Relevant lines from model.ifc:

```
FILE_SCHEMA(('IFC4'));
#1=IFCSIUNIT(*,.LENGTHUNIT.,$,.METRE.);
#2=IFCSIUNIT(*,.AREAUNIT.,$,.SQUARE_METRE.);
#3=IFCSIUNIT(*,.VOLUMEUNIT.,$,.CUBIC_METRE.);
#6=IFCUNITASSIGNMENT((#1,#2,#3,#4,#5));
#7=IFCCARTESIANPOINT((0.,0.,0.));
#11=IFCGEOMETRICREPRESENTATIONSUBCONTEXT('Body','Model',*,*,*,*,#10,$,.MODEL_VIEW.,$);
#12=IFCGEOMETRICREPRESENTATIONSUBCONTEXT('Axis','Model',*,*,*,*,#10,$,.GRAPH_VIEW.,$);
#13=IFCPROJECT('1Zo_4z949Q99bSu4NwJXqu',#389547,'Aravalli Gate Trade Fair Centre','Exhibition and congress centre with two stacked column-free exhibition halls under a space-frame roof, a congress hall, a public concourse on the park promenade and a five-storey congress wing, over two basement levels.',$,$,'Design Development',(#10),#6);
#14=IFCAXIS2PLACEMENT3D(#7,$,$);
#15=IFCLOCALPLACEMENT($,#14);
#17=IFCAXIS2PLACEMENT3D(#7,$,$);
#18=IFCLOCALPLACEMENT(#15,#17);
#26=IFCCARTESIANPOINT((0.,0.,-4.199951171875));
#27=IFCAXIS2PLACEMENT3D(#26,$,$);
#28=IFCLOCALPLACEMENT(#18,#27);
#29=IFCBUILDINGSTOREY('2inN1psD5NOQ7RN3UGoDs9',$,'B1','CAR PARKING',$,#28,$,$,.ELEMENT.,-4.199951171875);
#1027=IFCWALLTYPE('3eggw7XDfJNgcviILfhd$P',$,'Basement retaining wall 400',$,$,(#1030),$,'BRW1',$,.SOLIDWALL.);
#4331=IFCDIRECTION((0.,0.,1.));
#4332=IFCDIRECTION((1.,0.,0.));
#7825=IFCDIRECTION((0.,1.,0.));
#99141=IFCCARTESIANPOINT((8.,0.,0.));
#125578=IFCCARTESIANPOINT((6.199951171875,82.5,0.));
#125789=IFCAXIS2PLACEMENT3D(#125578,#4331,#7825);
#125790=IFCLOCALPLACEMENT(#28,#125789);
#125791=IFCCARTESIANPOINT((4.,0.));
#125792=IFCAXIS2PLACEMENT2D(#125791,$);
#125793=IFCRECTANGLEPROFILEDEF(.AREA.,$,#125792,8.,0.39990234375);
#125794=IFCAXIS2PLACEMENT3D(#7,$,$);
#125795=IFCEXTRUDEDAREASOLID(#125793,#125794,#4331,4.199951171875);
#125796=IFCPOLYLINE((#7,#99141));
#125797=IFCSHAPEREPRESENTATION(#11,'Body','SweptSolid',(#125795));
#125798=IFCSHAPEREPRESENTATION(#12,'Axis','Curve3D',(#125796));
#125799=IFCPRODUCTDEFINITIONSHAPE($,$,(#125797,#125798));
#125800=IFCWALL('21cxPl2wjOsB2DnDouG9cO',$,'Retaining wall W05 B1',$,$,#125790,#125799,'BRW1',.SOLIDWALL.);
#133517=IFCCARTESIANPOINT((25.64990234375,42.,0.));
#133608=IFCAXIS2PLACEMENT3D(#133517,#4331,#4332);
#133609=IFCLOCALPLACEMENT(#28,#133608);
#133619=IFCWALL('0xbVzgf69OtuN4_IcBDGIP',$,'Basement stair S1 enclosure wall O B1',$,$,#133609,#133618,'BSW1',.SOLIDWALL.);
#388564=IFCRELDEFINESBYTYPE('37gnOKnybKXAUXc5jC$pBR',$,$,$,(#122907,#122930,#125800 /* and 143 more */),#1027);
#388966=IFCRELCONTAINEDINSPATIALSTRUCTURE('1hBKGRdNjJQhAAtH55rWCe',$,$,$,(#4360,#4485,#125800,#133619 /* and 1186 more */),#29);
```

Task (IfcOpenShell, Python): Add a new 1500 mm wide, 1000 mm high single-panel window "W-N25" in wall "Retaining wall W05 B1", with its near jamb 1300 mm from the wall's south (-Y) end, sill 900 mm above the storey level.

```python
import numpy as np
import ifcopenshell
import ifcopenshell.api.feature
import ifcopenshell.api.geometry
import ifcopenshell.api.root
import ifcopenshell.api.spatial
import ifcopenshell.geom
import ifcopenshell.util.element
import ifcopenshell.util.placement
import ifcopenshell.util.representation
import ifcopenshell.util.shape
import ifcopenshell.util.unit

model = ifcopenshell.open("model.ifc")
unit_scale = ifcopenshell.util.unit.calculate_unit_scale(model)
settings = ifcopenshell.geom.settings()


def volume(element):
    """Net volume in cubic metres, openings subtracted."""
    shape = ifcopenshell.geom.create_shape(settings, element)
    return ifcopenshell.util.shape.get_volume(shape.geometry)


wall = model.by_guid("21cxPl2wjOsB2DnDouG9cO")
storey = ifcopenshell.util.element.get_container(wall, ifc_class="IfcBuildingStorey")
context = ifcopenshell.util.representation.get_context(model, "Model", "Body", "MODEL_VIEW")
before = volume(wall)

width, height, from_end, sill = 1.5, 1, 1.3, 0.9  # metres

# The wall runs along its own X axis, and the end named is its -X end.
wall_shape = ifcopenshell.geom.create_shape(settings, wall)
x, y, z = ifcopenshell.util.shape.get_vertices(wall_shape.geometry).T
start = x.min() + from_end
face, thickness = float(y.min()), float(y.max() - y.min())
wall_matrix = ifcopenshell.util.placement.get_local_placement(wall.ObjectPlacement)
level = ifcopenshell.util.placement.get_local_placement(storey.ObjectPlacement)[2, 3]


def in_wall(x, y):
    """Placement at x, y metres in the wall's axes, at sill height."""
    matrix = wall_matrix.copy()
    matrix[:, 3] = wall_matrix @ np.array([x / unit_scale, y / unit_scale, 0.0, 1.0])
    matrix[2, 3] = level + sill / unit_scale
    return matrix


# Opening: a box that overshoots both wall faces by 50 mm.
opening = ifcopenshell.api.root.create_entity(model, ifc_class="IfcOpeningElement", predefined_type="OPENING")
box = ifcopenshell.api.geometry.add_wall_representation(
    model, context=context, length=width, height=height, thickness=thickness + 0.1
)
ifcopenshell.api.geometry.assign_representation(model, product=opening, representation=box)
ifcopenshell.api.geometry.edit_object_placement(model, product=opening, matrix=in_wall(start, face - 0.05), is_si=False)
ifcopenshell.api.feature.add_feature(model, feature=opening, element=wall)

window = ifcopenshell.api.root.create_entity(model, ifc_class="IfcWindow", name="W-N25", predefined_type="WINDOW")
window.OverallWidth, window.OverallHeight = width / unit_scale, height / unit_scale
window.PartitioningType = "SINGLE_PANEL"
body = ifcopenshell.api.geometry.add_window_representation(
    model,
    context=context,
    overall_width=window.OverallWidth,
    overall_height=window.OverallHeight,
    partition_type="SINGLE_PANEL",
)
ifcopenshell.api.geometry.assign_representation(model, product=window, representation=body)
ifcopenshell.api.spatial.assign_container(model, products=[window], relating_structure=storey)
ifcopenshell.api.feature.add_filling(model, opening=opening, element=window)

# Centre the window in the wall's thickness.
ifcopenshell.api.geometry.edit_object_placement(model, product=window, matrix=in_wall(start, face), is_si=False)
window_shape = ifcopenshell.geom.create_shape(settings, window)
depth = ifcopenshell.util.shape.get_vertices(window_shape.geometry)[:, 1]
offset = face + thickness / 2 - (depth.min() + depth.max()) / 2
ifcopenshell.api.geometry.edit_object_placement(model, product=window, matrix=in_wall(start, offset), is_si=False)

after = volume(wall)

print(f"wall volume {before:.3f} -> {after:.3f} m3")

model.write("model_rev.ifc")
```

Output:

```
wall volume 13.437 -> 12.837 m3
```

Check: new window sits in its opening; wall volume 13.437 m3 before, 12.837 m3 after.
